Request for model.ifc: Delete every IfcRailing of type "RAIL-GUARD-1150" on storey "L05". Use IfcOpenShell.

First a look at what the model holds.

```python
import ifcopenshell
import ifcopenshell.util.element

model = ifcopenshell.open("model.ifc")
print(model.schema)
storey = next(s for s in model.by_type("IfcBuildingStorey") if s.Name == "L05")
railings = [e for e in ifcopenshell.util.element.get_decomposition(storey) if e.is_a("IfcRailing")]
seen = {}
for e in railings:
    element_type = ifcopenshell.util.element.get_type(e)
    name = element_type.Name if element_type not in (None, e) else None
    seen[name] = seen.get(name, 0) + 1
for name, count in sorted(seen.items(), key=str):
    print(count, "x", name)
```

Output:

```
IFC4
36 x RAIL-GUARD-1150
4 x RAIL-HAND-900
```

```python
import ifcopenshell
import ifcopenshell.api.root
import ifcopenshell.util.element

model = ifcopenshell.open("model.ifc")

storey = next(s for s in model.by_type("IfcBuildingStorey") if s.Name == "L05")
railings = [e for e in ifcopenshell.util.element.get_decomposition(storey) if e.is_a("IfcRailing")]
targets = [e for e in railings if (t := ifcopenshell.util.element.get_type(e)) not in (None, e) and t.Name == "RAIL-GUARD-1150"]

for e in targets:
    ifcopenshell.api.root.remove_product(model, product=e)
print(len(targets), "removed")

model.write("model-out.ifc")
```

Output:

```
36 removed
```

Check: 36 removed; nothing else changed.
